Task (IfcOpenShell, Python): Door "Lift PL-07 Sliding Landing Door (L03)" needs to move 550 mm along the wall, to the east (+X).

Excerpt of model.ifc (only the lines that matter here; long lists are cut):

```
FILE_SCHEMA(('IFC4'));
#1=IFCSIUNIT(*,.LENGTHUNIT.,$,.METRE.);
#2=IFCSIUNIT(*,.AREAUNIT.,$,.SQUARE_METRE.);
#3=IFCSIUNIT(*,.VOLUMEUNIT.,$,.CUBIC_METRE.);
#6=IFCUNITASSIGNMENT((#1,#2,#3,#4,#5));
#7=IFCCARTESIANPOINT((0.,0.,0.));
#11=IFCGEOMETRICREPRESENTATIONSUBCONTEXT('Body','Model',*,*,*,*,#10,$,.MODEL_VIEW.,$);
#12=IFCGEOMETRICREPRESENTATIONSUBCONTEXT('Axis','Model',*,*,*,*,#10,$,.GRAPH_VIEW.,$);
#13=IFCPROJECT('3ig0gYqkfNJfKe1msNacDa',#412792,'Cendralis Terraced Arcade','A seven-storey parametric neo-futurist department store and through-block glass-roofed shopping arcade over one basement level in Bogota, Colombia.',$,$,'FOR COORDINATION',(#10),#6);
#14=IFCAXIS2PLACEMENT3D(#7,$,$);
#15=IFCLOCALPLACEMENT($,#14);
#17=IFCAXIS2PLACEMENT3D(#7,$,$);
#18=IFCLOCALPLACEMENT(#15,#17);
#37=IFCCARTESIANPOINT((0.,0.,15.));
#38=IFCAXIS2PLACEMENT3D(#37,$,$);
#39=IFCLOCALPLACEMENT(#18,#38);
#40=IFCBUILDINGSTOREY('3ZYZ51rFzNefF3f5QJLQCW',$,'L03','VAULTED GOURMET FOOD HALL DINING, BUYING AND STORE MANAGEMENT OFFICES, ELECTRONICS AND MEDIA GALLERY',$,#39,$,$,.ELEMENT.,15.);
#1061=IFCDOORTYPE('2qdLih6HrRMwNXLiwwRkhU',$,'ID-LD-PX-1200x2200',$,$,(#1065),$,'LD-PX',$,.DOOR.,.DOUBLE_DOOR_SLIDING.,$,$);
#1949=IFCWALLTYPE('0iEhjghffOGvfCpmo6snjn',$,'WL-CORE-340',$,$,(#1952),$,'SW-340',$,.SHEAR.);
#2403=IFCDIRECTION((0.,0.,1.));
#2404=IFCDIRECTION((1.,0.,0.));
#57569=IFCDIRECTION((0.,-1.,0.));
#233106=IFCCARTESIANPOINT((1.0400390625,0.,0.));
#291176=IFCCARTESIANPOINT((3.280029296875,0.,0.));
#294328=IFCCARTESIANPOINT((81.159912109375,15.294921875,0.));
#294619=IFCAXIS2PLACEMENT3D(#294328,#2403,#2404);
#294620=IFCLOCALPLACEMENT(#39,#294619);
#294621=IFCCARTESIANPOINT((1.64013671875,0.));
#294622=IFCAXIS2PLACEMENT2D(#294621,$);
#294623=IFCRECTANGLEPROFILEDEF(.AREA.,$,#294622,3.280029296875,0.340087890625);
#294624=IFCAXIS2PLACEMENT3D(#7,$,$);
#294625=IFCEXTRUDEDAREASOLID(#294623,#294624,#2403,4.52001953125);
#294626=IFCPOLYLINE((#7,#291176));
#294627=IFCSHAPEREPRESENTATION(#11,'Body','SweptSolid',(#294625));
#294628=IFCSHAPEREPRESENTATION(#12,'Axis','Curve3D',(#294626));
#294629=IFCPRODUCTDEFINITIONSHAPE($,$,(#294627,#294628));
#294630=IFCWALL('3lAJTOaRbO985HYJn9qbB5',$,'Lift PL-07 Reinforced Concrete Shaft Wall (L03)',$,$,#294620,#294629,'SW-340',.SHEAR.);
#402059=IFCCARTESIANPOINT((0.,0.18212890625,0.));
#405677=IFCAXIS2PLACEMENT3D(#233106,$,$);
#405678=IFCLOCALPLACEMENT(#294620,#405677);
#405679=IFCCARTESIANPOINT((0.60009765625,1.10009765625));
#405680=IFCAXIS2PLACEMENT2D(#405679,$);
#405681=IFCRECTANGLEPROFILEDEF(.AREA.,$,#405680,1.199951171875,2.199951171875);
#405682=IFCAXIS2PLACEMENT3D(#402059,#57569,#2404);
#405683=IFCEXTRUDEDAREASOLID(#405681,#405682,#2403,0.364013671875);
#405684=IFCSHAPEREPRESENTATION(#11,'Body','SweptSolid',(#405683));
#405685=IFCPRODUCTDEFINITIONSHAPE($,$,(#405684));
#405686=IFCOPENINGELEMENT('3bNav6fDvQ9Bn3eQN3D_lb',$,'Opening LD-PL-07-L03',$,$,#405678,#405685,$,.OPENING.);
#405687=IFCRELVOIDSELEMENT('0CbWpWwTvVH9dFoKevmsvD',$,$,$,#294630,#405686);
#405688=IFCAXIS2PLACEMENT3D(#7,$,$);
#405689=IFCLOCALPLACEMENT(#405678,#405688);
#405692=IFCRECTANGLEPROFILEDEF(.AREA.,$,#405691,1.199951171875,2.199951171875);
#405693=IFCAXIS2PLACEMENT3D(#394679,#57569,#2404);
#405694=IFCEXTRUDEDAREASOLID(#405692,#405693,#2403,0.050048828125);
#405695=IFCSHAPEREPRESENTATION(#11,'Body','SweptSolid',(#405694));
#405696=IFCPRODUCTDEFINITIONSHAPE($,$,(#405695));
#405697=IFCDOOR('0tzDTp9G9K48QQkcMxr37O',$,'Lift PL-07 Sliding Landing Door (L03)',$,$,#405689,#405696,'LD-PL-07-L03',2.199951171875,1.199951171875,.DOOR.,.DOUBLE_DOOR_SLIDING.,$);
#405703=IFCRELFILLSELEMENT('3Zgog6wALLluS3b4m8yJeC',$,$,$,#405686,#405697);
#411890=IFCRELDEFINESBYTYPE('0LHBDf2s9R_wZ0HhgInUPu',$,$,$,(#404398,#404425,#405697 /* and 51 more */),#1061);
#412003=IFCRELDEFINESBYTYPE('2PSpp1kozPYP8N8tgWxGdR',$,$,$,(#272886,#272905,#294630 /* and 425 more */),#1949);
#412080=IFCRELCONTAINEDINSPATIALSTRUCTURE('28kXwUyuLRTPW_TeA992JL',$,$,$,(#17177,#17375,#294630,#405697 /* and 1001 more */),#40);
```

```python
import ifcopenshell
import ifcopenshell.api.geometry
import ifcopenshell.util.placement
import ifcopenshell.util.unit

model = ifcopenshell.open("model.ifc")
unit_scale = ifcopenshell.util.unit.calculate_unit_scale(model)

door = model.by_guid("0tzDTp9G9K48QQkcMxr37O")
opening = door.FillsVoids[0].RelatingOpeningElement
wall = opening.VoidsElements[0].RelatingBuildingElement

wall_matrix = ifcopenshell.util.placement.get_local_placement(wall.ObjectPlacement)
shift = wall_matrix[:3, 0] * 0.55 / unit_scale
before = ifcopenshell.util.placement.get_local_placement(door.ObjectPlacement)[:3, 3].copy()

# The door is placed relative to its opening, so it follows when the opening moves.
matrix = ifcopenshell.util.placement.get_local_placement(opening.ObjectPlacement)
matrix[:3, 3] += shift
ifcopenshell.api.geometry.edit_object_placement(
    model, product=opening, matrix=matrix, is_si=False, should_transform_children=True
)

after = ifcopenshell.util.placement.get_local_placement(door.ObjectPlacement)[:3, 3]
print("door moved by", (after - before).round(3) + 0.0)

model.write("model_updated.ifc")
```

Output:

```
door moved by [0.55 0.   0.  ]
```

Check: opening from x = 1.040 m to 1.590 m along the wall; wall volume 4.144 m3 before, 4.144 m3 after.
